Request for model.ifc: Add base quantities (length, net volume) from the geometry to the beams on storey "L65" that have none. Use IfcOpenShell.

First a look at what the model holds.

```python
import ifcopenshell
import ifcopenshell.util.element
import ifcopenshell.util.unit

model = ifcopenshell.open("model.ifc")
print(model.schema)
for unit_type in ("LENGTHUNIT", "AREAUNIT", "VOLUMEUNIT"):
    print(unit_type, ifcopenshell.util.unit.calculate_unit_scale(model, unit_type))
storey = next(s for s in model.by_type("IfcBuildingStorey") if s.Name == "L65")
beams = [e for e in ifcopenshell.util.element.get_decomposition(storey) if e.is_a("IfcBeam")]
for e in sorted(beams, key=lambda e: e.id()):
    print(e.id(), e.is_a(), e.Name, list(ifcopenshell.util.element.get_psets(e, qtos_only=True)), sep=" | ")
```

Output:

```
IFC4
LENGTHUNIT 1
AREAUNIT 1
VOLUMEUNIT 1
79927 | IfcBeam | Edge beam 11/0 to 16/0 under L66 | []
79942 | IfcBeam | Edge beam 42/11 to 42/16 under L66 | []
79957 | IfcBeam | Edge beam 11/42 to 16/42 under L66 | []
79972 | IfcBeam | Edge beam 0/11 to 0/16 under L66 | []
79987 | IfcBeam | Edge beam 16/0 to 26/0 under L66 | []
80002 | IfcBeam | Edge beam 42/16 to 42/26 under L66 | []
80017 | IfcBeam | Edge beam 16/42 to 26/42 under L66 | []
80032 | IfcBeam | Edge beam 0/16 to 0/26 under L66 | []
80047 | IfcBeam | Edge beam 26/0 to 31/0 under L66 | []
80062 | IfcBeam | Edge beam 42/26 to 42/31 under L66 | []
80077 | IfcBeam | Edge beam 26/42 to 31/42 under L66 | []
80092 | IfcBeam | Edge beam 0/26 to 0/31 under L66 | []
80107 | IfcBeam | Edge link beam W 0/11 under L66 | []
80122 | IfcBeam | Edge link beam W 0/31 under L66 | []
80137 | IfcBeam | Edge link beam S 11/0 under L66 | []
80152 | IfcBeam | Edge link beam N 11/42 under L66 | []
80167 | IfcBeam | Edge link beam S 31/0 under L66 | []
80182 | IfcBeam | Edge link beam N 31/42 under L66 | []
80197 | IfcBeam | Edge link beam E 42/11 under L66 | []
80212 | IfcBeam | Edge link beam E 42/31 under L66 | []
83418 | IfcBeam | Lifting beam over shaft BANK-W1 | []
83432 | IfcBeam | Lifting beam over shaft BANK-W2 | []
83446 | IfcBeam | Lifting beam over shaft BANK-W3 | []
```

```python
import ifcopenshell
import ifcopenshell.api.pset
import ifcopenshell.geom
import ifcopenshell.util.element
import ifcopenshell.util.shape
import ifcopenshell.util.unit

model = ifcopenshell.open("model.ifc")
unit_scale = ifcopenshell.util.unit.calculate_unit_scale(model)
volume_scale = ifcopenshell.util.unit.calculate_unit_scale(model, "VOLUMEUNIT")
settings = ifcopenshell.geom.settings()

storey = next(s for s in model.by_type("IfcBuildingStorey") if s.Name == "L65")
beams = [e for e in ifcopenshell.util.element.get_decomposition(storey) if e.is_a("IfcBeam")]

for e in sorted(beams, key=lambda e: e.id()):
    if ifcopenshell.util.element.get_psets(e, qtos_only=True, should_inherit=False):
        continue
    # Geometry comes back in metres, in the element's own axes.
    shape = ifcopenshell.geom.create_shape(settings, e)
    values = {
        "Length": ifcopenshell.util.shape.get_max_xyz(shape.geometry) / unit_scale,
        "NetVolume": ifcopenshell.util.shape.get_volume(shape.geometry) / volume_scale,
    }
    qto = ifcopenshell.api.pset.add_qto(model, product=e, name="Qto_BeamBaseQuantities")
    ifcopenshell.api.pset.edit_qto(model, qto=qto, properties=values)
    print(e.id(), {k: round(v, 3) for k, v in values.items()})

model.write("model_v2.ifc")
```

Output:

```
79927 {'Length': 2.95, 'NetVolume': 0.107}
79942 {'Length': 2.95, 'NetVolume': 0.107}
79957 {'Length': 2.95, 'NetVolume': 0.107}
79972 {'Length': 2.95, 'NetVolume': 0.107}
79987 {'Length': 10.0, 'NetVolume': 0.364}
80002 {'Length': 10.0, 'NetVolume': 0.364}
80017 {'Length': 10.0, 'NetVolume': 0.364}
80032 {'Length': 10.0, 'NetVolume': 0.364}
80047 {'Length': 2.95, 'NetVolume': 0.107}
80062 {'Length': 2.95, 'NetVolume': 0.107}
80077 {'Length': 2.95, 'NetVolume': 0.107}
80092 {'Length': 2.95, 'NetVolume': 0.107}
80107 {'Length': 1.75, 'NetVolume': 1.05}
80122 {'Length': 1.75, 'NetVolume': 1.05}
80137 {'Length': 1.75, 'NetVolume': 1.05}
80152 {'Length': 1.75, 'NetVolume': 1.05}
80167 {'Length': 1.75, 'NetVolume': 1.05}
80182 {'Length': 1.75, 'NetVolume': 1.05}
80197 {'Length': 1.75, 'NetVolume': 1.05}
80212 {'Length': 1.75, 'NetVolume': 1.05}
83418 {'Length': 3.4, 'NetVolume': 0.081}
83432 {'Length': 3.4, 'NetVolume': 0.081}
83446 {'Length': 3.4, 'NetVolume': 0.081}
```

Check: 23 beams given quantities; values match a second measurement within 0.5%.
